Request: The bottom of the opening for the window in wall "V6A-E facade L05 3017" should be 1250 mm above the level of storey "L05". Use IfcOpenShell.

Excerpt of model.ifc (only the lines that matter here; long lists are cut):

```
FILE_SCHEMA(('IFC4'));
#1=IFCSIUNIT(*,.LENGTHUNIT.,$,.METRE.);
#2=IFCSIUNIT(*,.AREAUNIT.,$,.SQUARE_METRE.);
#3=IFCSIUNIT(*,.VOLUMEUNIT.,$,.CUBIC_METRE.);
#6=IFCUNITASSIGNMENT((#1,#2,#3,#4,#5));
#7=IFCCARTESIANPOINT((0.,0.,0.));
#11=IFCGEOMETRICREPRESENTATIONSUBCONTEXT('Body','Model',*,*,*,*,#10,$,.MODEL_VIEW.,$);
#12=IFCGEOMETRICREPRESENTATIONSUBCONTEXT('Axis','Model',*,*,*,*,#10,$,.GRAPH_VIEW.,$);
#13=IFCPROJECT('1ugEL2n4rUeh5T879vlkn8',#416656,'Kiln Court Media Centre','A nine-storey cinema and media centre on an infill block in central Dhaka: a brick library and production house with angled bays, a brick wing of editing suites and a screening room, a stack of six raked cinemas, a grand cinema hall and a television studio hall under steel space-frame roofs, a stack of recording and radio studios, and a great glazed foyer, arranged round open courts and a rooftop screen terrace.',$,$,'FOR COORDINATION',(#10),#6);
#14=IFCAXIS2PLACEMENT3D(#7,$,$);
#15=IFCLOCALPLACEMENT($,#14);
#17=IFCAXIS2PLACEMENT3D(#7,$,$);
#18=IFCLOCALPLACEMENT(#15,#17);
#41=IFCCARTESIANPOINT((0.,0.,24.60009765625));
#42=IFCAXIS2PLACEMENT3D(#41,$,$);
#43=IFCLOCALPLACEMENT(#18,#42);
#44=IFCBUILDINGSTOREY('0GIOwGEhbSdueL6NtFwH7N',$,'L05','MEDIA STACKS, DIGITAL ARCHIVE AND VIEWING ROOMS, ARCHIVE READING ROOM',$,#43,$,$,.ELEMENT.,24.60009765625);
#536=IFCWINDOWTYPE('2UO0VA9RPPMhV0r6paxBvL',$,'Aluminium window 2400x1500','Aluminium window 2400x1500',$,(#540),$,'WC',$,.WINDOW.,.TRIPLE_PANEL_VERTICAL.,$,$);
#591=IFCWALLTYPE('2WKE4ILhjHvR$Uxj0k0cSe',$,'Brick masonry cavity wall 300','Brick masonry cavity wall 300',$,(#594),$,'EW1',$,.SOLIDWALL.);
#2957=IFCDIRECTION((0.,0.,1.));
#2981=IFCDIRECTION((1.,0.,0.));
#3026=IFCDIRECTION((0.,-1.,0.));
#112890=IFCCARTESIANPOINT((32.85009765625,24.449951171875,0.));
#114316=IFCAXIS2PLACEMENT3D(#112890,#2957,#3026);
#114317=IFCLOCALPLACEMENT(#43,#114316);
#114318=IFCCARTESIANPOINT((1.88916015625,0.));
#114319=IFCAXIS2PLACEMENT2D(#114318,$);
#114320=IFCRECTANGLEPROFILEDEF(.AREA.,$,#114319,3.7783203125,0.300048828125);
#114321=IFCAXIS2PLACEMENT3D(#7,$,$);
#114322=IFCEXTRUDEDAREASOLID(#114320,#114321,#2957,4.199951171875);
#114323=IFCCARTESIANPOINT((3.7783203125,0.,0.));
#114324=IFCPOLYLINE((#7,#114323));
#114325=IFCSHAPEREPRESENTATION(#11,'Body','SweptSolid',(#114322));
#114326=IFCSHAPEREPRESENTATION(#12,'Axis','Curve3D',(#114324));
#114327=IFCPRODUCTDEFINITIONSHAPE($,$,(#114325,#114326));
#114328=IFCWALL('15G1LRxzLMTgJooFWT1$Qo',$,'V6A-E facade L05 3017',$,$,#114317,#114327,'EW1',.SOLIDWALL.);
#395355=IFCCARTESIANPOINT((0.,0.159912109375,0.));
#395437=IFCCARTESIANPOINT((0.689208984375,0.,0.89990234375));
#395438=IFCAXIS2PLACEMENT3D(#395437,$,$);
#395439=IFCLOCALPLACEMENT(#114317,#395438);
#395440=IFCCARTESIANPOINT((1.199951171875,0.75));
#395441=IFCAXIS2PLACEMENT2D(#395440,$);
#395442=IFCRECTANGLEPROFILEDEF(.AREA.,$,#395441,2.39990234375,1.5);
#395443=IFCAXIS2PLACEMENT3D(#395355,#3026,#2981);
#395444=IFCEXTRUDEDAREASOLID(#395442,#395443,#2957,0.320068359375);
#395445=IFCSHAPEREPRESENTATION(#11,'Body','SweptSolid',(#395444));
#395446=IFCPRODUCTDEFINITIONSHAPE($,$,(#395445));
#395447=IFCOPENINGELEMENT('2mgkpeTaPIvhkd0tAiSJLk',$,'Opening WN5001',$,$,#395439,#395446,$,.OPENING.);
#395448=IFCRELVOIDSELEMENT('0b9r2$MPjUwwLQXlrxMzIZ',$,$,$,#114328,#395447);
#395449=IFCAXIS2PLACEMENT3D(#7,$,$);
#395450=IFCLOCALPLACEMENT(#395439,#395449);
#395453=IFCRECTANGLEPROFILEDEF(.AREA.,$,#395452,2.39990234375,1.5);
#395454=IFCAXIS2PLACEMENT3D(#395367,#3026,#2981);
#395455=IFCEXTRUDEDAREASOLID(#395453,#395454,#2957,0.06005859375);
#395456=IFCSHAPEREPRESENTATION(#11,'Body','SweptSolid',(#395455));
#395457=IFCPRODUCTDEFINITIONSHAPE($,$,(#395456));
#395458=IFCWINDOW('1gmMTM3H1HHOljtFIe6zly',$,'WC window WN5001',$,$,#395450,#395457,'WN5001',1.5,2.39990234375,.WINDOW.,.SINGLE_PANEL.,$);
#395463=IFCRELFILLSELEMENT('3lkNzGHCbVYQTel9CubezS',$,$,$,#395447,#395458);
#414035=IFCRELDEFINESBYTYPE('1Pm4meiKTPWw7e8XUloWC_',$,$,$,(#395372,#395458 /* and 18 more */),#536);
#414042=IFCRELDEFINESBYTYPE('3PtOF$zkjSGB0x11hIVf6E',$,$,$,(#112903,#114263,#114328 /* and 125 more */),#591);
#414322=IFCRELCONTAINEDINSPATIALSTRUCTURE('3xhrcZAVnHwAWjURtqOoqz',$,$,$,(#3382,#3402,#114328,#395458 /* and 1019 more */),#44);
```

```python
import numpy as np
import ifcopenshell
import ifcopenshell.api.geometry
import ifcopenshell.geom
import ifcopenshell.util.element
import ifcopenshell.util.placement
import ifcopenshell.util.shape
import ifcopenshell.util.unit

model = ifcopenshell.open("model.ifc")
unit_scale = ifcopenshell.util.unit.calculate_unit_scale(model)

window = model.by_guid("1gmMTM3H1HHOljtFIe6zly")
opening = window.FillsVoids[0].RelatingOpeningElement
storey = ifcopenshell.util.element.get_container(window, ifc_class="IfcBuildingStorey")
level = ifcopenshell.util.placement.get_local_placement(storey.ObjectPlacement)[2, 3]

# The opening's origin need not be at the sill, so measure its lowest point.
shape = ifcopenshell.geom.create_shape(ifcopenshell.geom.settings(), opening)
bottom = ifcopenshell.util.shape.get_shape_bottom_elevation(shape, shape.geometry) / unit_scale
dz = level + 1.25 - bottom

shift = np.array([0.0, 0.0, dz])
# The window is placed relative to its opening, so it follows when the opening moves.
matrix = ifcopenshell.util.placement.get_local_placement(opening.ObjectPlacement)
matrix[:3, 3] += shift
ifcopenshell.api.geometry.edit_object_placement(
    model, product=opening, matrix=matrix, is_si=False, should_transform_children=True
)

print(f"moved by {dz * unit_scale:+.3f} m")

model.write("model_updated.ifc")
```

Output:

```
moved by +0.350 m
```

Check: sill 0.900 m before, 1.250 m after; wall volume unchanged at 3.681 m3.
